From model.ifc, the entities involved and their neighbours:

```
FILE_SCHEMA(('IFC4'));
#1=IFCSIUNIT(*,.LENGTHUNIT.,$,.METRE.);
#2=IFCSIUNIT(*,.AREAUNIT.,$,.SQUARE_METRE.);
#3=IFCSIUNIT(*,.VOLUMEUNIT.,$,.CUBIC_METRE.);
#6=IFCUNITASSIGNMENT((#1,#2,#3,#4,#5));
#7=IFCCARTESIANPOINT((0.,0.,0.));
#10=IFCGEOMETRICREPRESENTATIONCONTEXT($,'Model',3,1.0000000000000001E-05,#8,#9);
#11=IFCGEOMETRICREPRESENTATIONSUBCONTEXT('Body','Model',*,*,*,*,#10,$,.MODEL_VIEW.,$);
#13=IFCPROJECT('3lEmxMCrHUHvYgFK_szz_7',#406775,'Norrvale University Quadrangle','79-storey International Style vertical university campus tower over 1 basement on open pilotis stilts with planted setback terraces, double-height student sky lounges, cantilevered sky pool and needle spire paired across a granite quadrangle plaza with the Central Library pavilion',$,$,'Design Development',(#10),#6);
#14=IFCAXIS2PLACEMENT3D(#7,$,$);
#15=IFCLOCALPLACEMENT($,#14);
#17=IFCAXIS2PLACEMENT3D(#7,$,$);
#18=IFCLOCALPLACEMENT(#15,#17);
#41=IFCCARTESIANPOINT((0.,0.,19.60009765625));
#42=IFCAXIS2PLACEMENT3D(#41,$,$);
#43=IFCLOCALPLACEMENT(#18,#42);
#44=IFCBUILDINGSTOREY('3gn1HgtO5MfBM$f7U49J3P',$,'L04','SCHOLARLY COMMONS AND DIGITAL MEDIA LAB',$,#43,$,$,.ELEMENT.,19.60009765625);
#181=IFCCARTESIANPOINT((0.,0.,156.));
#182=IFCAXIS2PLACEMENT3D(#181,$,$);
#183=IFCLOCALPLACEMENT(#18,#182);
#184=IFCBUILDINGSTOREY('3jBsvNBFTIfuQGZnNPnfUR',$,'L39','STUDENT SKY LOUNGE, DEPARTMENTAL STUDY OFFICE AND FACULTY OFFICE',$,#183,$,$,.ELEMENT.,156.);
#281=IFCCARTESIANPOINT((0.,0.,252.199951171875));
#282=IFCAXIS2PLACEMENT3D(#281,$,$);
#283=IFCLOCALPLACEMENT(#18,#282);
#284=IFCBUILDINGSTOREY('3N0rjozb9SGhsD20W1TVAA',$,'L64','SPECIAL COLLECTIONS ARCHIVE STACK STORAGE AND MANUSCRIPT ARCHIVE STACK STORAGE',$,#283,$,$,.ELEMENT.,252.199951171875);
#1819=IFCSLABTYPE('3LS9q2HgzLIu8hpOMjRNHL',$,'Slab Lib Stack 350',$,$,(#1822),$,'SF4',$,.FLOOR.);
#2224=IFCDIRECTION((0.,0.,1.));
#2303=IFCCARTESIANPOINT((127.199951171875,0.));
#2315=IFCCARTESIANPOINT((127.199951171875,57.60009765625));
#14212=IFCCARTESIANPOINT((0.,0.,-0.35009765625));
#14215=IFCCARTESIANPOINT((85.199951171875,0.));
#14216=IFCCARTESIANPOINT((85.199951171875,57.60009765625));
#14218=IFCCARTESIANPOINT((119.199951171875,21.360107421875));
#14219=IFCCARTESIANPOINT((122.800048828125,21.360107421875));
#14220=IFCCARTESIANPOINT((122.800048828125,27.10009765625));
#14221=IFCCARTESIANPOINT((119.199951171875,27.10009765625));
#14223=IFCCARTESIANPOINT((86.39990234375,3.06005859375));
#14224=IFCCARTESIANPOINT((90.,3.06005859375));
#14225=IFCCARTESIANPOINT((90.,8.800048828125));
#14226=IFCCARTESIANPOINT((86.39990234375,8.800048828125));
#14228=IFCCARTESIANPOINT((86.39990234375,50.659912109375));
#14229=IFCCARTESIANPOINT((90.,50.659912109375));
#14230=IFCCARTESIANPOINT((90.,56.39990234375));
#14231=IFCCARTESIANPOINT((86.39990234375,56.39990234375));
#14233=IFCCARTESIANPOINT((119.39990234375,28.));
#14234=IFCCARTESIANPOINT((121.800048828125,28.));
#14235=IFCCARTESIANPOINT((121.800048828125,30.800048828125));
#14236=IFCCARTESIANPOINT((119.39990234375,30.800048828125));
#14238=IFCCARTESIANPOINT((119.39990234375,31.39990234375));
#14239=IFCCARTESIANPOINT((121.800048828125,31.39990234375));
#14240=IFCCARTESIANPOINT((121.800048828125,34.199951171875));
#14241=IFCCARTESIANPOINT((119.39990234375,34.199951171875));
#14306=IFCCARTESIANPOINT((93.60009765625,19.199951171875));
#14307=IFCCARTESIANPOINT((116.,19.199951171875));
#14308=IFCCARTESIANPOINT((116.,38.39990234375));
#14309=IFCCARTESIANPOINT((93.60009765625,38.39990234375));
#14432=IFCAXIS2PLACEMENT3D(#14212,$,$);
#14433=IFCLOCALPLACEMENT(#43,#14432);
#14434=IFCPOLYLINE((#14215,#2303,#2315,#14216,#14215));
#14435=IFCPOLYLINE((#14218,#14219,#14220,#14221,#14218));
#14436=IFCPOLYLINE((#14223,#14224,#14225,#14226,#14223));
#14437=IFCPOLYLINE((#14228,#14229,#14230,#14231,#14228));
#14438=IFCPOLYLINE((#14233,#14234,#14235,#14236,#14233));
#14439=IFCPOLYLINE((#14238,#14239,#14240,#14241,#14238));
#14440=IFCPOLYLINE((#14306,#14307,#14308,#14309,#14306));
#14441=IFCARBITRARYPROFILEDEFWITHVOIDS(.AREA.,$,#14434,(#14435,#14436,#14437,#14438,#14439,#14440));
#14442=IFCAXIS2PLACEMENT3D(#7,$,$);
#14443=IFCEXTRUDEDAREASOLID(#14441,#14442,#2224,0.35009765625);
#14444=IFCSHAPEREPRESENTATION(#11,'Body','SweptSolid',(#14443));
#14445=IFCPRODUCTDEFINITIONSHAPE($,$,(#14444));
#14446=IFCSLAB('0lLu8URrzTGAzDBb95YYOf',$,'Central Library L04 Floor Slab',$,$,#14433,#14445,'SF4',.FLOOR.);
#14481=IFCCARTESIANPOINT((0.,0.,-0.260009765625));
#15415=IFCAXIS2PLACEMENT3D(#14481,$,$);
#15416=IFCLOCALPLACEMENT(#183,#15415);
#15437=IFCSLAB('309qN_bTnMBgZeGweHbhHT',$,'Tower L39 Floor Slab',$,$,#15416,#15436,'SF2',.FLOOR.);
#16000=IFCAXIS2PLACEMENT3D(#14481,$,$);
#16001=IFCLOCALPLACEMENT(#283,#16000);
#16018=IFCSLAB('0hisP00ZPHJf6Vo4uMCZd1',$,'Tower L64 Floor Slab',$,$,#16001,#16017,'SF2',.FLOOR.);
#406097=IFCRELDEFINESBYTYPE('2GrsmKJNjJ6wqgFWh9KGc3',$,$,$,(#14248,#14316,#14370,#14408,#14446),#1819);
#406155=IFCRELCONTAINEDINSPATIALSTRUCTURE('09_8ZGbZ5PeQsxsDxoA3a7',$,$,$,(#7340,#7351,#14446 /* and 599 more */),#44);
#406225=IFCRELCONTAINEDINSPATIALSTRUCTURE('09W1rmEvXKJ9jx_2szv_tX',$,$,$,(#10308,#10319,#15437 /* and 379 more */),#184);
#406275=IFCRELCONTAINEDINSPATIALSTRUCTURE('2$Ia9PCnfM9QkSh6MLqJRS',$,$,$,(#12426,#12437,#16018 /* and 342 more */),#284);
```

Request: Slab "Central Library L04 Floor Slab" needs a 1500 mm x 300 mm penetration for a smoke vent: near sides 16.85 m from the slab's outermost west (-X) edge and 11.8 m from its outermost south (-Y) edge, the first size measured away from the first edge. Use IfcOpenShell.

```python
import numpy as np
import ifcopenshell
import ifcopenshell.api.feature
import ifcopenshell.api.geometry
import ifcopenshell.api.root
import ifcopenshell.geom
import ifcopenshell.util.placement
import ifcopenshell.util.representation
import ifcopenshell.util.shape
import ifcopenshell.util.unit

model = ifcopenshell.open("model.ifc")
unit_scale = ifcopenshell.util.unit.calculate_unit_scale(model)
settings = ifcopenshell.geom.settings()


def volume(element):
    """Net volume in cubic metres, openings subtracted."""
    shape = ifcopenshell.geom.create_shape(settings, element)
    return ifcopenshell.util.shape.get_volume(shape.geometry)


slab = model.by_id(14446)
before = volume(slab)

# Extent in the slab's own axes, in metres. The edges named are its -X and -Y sides.
slab_shape = ifcopenshell.geom.create_shape(settings, slab)
vertices = ifcopenshell.util.shape.get_vertices(slab_shape.geometry)
x_min, y_min, bottom = vertices.min(axis=0)
top = vertices[:, 2].max()

opening = ifcopenshell.api.root.create_entity(model, ifc_class="IfcOpeningElement", name="Smoke vent opening", predefined_type="OPENING")
context = ifcopenshell.util.representation.get_context(model, "Model", "Body", "MODEL_VIEW")
width, depth = 1.5, 0.3
outline = [(0.0, 0.0), (width, 0.0), (width, depth), (0.0, depth), (0.0, 0.0)]
# Overshoot both faces by 50 mm so the cut is clean.
shape = ifcopenshell.api.geometry.add_slab_representation(
    model, context=context, depth=top - bottom + 0.1, polyline=outline
)
ifcopenshell.api.geometry.assign_representation(model, product=opening, representation=shape)

matrix = ifcopenshell.util.placement.get_local_placement(slab.ObjectPlacement)
matrix[:, 3] = matrix @ np.append(np.array([x_min + 16.85, y_min + 11.8, bottom - 0.05]) / unit_scale, 1.0)
ifcopenshell.api.geometry.edit_object_placement(model, product=opening, matrix=matrix, is_si=False)
ifcopenshell.api.feature.add_feature(model, feature=opening, element=slab)

after = volume(slab)

print(f"slab volume {before:.3f} -> {after:.3f} m3")

model.write("model_edited.ifc")
```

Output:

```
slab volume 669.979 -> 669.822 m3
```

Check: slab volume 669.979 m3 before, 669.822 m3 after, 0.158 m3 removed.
